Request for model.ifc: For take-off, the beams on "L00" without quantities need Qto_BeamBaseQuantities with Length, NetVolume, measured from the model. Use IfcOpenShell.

First a look at what the model holds.

```python
import ifcopenshell
import ifcopenshell.util.element
import ifcopenshell.util.unit

model = ifcopenshell.open("model.ifc")
print(model.schema)
for unit_type in ("LENGTHUNIT", "AREAUNIT", "VOLUMEUNIT"):
    print(unit_type, ifcopenshell.util.unit.calculate_unit_scale(model, unit_type))
storey = next(s for s in model.by_type("IfcBuildingStorey") if s.Name == "L00")
beams = [e for e in ifcopenshell.util.element.get_decomposition(storey) if e.is_a("IfcBeam")]
for e in sorted(beams, key=lambda e: e.id()):
    print(e.id(), e.is_a(), e.Name, list(ifcopenshell.util.element.get_psets(e, qtos_only=True)), sep=" | ")
```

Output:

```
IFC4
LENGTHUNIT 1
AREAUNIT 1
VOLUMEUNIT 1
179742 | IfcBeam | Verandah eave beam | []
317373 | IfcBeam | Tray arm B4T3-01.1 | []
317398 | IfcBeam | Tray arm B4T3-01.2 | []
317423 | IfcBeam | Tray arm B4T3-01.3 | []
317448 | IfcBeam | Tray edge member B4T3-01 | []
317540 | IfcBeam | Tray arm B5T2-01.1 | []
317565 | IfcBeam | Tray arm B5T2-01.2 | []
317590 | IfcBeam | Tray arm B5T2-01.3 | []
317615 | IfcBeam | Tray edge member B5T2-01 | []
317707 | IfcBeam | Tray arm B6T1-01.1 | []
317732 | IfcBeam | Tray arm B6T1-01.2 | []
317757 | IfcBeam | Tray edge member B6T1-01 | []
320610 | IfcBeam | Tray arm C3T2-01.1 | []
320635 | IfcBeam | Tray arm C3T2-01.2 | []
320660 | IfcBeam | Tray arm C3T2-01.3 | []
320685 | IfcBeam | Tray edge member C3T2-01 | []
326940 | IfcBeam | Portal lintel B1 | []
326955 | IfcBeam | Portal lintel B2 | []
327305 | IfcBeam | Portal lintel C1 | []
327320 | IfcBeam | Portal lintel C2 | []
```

```python
import ifcopenshell
import ifcopenshell.api.pset
import ifcopenshell.geom
import ifcopenshell.util.element
import ifcopenshell.util.shape
import ifcopenshell.util.unit

model = ifcopenshell.open("model.ifc")
unit_scale = ifcopenshell.util.unit.calculate_unit_scale(model)
volume_scale = ifcopenshell.util.unit.calculate_unit_scale(model, "VOLUMEUNIT")
settings = ifcopenshell.geom.settings()

storey = next(s for s in model.by_type("IfcBuildingStorey") if s.Name == "L00")
beams = [e for e in ifcopenshell.util.element.get_decomposition(storey) if e.is_a("IfcBeam")]

for e in sorted(beams, key=lambda e: e.id()):
    if ifcopenshell.util.element.get_psets(e, qtos_only=True, should_inherit=False):
        continue
    # Geometry comes back in metres, in the element's own axes.
    shape = ifcopenshell.geom.create_shape(settings, e)
    values = {
        "Length": ifcopenshell.util.shape.get_max_xyz(shape.geometry) / unit_scale,
        "NetVolume": ifcopenshell.util.shape.get_volume(shape.geometry) / volume_scale,
    }
    qto = ifcopenshell.api.pset.add_qto(model, product=e, name="Qto_BeamBaseQuantities")
    ifcopenshell.api.pset.edit_qto(model, qto=qto, properties=values)
    print(e.id(), {k: round(v, 3) for k, v in values.items()})

model.write("model_updated.ifc")
```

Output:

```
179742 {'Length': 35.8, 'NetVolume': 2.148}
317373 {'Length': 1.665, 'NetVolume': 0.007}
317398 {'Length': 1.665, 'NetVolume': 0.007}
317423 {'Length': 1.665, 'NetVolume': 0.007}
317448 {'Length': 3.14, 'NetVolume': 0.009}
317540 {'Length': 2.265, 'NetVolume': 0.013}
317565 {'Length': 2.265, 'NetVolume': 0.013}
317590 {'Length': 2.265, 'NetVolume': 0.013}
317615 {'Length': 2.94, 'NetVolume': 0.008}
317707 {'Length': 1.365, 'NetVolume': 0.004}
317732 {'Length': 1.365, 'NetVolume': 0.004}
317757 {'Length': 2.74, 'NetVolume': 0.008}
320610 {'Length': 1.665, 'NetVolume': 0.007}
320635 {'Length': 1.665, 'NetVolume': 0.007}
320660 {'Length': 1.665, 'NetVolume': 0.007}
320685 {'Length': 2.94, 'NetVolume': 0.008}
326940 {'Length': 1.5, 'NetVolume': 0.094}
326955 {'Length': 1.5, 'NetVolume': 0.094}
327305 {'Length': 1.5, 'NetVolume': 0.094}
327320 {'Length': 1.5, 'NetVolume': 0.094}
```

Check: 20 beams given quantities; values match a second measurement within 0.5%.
